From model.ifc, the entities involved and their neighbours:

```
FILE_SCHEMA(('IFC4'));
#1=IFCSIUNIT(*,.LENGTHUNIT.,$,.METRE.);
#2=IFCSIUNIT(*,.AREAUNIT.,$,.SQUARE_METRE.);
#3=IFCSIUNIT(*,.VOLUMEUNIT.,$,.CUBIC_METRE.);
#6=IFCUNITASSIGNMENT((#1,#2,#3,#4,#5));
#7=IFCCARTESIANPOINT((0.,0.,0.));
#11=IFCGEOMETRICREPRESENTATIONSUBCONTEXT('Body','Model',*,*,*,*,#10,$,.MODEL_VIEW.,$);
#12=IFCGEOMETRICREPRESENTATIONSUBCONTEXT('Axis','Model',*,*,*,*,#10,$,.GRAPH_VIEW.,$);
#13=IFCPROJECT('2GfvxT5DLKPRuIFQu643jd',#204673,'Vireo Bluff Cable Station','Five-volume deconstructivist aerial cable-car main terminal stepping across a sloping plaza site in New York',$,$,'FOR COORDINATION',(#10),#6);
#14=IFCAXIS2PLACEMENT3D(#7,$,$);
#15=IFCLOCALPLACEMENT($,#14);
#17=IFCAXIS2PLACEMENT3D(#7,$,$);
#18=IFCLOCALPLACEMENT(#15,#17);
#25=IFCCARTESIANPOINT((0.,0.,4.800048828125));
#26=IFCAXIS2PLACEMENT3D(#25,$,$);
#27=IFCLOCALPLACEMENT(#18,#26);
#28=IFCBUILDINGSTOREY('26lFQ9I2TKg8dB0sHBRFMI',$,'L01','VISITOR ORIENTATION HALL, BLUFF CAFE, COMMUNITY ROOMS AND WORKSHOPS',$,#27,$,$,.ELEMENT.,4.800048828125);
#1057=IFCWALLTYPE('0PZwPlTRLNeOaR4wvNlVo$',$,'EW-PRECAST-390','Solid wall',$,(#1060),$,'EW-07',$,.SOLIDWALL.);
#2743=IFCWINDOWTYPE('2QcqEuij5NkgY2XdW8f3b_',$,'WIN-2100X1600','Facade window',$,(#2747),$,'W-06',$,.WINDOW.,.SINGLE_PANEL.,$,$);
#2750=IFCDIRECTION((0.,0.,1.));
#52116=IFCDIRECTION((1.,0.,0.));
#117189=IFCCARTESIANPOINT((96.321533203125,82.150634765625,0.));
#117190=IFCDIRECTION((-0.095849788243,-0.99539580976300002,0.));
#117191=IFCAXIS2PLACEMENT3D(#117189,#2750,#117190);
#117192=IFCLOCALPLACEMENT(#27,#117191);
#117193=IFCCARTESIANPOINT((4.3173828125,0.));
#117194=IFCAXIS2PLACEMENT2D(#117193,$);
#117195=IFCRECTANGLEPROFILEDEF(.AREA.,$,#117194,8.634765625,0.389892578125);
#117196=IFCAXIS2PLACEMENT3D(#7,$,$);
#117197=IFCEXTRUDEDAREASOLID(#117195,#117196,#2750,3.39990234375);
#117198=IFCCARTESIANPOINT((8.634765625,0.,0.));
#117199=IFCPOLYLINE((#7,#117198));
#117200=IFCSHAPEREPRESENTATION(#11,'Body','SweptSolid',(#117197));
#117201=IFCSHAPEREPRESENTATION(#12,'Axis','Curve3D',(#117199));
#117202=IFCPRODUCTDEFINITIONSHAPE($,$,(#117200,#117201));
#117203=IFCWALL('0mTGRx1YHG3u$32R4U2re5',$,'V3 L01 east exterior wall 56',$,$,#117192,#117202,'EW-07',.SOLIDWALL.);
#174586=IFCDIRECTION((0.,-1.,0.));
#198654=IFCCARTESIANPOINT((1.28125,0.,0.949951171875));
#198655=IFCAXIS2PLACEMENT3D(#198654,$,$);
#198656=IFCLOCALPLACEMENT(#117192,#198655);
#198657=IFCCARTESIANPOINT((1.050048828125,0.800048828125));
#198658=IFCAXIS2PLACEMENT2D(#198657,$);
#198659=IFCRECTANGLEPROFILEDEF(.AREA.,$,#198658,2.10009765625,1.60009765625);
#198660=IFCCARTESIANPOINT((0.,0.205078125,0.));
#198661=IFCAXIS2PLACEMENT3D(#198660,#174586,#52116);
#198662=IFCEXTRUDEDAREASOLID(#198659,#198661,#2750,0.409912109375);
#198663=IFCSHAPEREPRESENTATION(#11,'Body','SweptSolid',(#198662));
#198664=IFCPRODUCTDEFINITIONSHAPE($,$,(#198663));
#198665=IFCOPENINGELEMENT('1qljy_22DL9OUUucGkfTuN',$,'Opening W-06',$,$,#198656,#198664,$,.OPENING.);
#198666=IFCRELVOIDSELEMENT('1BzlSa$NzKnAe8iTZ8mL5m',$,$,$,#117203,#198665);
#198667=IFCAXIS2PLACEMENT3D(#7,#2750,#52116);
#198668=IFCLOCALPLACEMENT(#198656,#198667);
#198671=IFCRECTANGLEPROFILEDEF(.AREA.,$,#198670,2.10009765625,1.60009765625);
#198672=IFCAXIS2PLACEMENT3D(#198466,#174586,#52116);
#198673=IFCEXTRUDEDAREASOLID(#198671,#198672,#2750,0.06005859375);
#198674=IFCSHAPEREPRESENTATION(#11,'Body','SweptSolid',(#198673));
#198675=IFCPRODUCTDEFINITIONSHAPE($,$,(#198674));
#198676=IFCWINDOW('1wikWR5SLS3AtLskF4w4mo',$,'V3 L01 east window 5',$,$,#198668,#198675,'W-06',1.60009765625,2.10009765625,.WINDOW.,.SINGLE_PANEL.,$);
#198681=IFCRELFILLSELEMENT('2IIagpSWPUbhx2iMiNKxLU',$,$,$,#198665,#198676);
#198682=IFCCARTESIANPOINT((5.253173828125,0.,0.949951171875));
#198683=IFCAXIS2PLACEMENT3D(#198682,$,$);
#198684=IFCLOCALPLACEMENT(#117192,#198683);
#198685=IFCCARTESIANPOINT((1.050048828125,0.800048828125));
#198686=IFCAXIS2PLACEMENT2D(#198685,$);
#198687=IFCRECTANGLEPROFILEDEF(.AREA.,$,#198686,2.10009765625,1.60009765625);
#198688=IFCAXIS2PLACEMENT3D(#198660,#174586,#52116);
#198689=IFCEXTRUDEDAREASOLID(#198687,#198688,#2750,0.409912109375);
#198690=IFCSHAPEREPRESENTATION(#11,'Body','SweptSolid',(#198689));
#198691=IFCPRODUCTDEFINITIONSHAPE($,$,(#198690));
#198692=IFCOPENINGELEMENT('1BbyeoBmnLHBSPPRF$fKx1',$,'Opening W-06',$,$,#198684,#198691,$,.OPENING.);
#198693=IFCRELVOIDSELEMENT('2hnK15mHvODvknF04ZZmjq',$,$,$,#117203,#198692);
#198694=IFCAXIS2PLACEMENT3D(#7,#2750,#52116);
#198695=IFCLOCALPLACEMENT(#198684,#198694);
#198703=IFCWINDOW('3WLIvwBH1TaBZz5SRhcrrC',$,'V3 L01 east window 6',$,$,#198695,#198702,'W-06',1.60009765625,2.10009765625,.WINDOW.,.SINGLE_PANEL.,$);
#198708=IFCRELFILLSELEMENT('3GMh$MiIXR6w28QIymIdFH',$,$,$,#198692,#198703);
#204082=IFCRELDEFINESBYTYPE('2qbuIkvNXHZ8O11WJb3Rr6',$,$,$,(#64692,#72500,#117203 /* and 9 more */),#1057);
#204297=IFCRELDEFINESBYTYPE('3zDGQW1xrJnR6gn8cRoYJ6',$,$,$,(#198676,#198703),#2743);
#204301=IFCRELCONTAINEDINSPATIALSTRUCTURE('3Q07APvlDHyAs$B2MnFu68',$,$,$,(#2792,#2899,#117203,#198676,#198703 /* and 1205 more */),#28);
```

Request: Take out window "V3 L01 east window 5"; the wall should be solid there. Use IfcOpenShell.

```python
import ifcopenshell
import ifcopenshell.api.feature
import ifcopenshell.api.root
import ifcopenshell.geom
import ifcopenshell.util.shape

model = ifcopenshell.open("model.ifc")
settings = ifcopenshell.geom.settings()


def volume(element):
    """Net volume in cubic metres, openings subtracted."""
    shape = ifcopenshell.geom.create_shape(settings, element)
    return ifcopenshell.util.shape.get_volume(shape.geometry)


window = model.by_id(198676)
opening = window.FillsVoids[0].RelatingOpeningElement
wall = opening.VoidsElements[0].RelatingBuildingElement
before = volume(wall)

ifcopenshell.api.root.remove_product(model, product=window)
ifcopenshell.api.feature.remove_feature(model, feature=opening)

after = volume(wall)

print(f"wall volume {before:.3f} -> {after:.3f} m3")

model.write("model_v2.ifc")
```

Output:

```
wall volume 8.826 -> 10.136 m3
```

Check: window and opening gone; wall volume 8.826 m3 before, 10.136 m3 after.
